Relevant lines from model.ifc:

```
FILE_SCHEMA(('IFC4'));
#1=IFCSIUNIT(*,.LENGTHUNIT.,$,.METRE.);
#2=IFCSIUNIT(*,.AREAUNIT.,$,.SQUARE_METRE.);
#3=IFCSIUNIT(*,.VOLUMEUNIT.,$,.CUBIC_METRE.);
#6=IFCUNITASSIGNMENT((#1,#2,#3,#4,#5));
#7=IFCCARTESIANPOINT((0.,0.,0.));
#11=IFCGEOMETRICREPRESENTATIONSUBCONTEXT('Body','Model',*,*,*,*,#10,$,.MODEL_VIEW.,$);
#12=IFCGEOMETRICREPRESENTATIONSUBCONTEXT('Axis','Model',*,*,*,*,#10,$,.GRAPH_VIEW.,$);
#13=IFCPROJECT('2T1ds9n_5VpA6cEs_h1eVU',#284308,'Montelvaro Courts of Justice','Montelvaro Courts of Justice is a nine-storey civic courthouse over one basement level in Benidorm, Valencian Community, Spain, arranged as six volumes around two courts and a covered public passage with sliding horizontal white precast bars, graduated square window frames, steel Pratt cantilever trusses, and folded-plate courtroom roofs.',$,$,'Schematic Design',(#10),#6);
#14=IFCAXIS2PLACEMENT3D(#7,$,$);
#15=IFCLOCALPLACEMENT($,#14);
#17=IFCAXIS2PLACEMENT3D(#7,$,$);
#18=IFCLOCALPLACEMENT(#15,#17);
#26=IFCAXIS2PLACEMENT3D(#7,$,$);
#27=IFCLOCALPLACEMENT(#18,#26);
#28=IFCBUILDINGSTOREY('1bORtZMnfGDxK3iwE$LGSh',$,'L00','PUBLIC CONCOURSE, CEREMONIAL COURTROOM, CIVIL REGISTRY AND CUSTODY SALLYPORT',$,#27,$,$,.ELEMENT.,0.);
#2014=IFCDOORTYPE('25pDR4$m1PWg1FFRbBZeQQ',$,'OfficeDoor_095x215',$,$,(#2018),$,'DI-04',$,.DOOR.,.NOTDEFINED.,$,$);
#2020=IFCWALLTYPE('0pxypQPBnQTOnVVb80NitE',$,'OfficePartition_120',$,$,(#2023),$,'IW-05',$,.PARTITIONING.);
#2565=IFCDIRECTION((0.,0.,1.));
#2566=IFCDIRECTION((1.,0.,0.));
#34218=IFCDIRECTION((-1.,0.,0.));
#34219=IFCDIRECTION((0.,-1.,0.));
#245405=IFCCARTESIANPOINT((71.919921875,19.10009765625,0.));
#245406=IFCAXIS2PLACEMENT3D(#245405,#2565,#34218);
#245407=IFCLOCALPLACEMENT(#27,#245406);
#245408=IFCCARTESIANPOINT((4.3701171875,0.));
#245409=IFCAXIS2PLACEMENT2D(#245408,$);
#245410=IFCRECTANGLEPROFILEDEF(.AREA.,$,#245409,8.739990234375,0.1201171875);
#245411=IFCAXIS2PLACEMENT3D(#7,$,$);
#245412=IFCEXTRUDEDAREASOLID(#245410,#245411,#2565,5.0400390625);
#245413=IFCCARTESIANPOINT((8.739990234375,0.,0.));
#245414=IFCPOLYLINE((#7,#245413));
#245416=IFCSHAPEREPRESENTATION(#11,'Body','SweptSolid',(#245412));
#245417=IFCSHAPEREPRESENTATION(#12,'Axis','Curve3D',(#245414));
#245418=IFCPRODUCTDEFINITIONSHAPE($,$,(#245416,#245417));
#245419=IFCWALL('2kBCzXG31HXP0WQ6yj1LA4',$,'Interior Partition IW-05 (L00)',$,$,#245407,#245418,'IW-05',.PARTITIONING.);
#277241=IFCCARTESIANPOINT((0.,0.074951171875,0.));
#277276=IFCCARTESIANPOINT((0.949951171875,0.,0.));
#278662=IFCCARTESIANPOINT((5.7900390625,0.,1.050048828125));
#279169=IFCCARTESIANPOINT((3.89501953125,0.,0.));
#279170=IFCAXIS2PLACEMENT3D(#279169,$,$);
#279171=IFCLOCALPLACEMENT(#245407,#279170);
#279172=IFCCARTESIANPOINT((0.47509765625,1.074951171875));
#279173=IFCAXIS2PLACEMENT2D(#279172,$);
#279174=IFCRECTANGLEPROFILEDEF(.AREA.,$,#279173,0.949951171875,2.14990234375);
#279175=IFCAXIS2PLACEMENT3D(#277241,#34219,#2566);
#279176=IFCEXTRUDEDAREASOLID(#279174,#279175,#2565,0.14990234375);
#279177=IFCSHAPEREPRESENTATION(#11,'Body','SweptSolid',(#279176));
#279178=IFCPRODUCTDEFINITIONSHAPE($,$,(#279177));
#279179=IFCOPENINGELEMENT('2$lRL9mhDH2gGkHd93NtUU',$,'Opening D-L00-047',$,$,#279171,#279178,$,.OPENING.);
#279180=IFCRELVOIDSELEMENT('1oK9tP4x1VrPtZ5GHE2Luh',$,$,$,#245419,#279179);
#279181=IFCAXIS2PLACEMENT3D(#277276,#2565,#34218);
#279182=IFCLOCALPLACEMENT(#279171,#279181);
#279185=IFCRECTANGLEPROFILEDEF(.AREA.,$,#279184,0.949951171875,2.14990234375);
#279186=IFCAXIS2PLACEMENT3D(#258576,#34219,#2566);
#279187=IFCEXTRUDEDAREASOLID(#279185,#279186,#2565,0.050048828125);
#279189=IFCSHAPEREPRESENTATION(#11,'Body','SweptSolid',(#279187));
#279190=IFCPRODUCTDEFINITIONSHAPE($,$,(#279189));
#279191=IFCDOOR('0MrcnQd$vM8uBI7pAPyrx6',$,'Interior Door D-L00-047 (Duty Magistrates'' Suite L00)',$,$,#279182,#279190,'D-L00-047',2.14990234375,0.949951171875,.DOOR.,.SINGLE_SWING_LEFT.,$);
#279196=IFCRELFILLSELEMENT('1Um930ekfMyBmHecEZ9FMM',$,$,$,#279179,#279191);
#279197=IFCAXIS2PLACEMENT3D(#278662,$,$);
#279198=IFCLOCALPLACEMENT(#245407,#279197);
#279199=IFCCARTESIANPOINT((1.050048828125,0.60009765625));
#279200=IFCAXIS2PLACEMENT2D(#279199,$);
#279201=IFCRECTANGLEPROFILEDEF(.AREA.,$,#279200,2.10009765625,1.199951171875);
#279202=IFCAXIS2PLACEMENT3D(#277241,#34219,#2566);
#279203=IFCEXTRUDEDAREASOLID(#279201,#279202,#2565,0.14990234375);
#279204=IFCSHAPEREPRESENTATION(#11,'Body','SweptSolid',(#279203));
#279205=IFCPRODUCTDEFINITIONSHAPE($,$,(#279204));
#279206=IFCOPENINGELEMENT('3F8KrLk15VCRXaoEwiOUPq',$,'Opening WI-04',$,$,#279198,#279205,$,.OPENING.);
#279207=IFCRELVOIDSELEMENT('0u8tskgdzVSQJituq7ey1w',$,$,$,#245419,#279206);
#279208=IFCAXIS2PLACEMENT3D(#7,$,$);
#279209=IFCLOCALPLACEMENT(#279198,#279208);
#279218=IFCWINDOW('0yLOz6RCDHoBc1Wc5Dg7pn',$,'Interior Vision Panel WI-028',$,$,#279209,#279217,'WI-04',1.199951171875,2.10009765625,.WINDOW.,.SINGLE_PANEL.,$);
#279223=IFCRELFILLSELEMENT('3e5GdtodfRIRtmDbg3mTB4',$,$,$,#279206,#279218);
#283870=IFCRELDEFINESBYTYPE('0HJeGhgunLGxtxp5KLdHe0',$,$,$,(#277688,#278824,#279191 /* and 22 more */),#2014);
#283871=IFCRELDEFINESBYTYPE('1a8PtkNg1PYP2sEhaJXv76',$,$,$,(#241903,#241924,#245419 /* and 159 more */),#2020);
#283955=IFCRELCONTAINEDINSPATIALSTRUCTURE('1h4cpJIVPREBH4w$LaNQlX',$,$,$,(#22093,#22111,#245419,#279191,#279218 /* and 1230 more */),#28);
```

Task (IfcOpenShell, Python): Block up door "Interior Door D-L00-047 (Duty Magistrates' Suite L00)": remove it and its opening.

```python
import ifcopenshell
import ifcopenshell.api.feature
import ifcopenshell.api.root
import ifcopenshell.geom
import ifcopenshell.util.shape

model = ifcopenshell.open("model.ifc")
settings = ifcopenshell.geom.settings()


def volume(element):
    """Net volume in cubic metres, openings subtracted."""
    shape = ifcopenshell.geom.create_shape(settings, element)
    return ifcopenshell.util.shape.get_volume(shape.geometry)


door = model.by_guid("0MrcnQd$vM8uBI7pAPyrx6")
opening = door.FillsVoids[0].RelatingOpeningElement
wall = opening.VoidsElements[0].RelatingBuildingElement
before = volume(wall)

ifcopenshell.api.root.remove_product(model, product=door)
ifcopenshell.api.feature.remove_feature(model, feature=opening)

after = volume(wall)

print(f"wall volume {before:.3f} -> {after:.3f} m3")

model.write("model_rev.ifc")
```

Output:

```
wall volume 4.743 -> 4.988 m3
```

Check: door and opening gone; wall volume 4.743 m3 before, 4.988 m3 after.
